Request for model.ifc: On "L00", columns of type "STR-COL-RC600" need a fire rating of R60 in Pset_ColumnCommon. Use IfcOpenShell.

First a look at what the model holds.

```python
import ifcopenshell
import ifcopenshell.util.element

model = ifcopenshell.open("model.ifc")
print(model.schema)
storey = next(s for s in model.by_type("IfcBuildingStorey") if s.Name == "L00")
columns = [e for e in ifcopenshell.util.element.get_decomposition(storey) if e.is_a("IfcColumn")]
seen = {}
for e in columns:
    element_type = ifcopenshell.util.element.get_type(e)
    key = (element_type.Name if element_type != e and element_type else None, ifcopenshell.util.element.get_pset(e, "Pset_ColumnCommon", "FireRating"))
    seen[key] = seen.get(key, 0) + 1
for (name, value), count in sorted(seen.items(), key=str):
    print(count, "x", name, "|", value)
```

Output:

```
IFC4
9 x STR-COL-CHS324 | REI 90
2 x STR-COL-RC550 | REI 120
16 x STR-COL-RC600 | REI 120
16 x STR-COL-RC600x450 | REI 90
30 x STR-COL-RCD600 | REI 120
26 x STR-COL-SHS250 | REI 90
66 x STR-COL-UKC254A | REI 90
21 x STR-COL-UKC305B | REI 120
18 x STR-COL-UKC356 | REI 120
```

```python
import ifcopenshell
import ifcopenshell.api.pset
import ifcopenshell.util.element

model = ifcopenshell.open("model.ifc")

storey = next(s for s in model.by_type("IfcBuildingStorey") if s.Name == "L00")
columns = [e for e in ifcopenshell.util.element.get_decomposition(storey) if e.is_a("IfcColumn")]

count = 0
for e in columns:
    element_type = ifcopenshell.util.element.get_type(e)
    if element_type in (None, e) or element_type.Name != "STR-COL-RC600":
        continue
    # add_pset returns the element's existing set when there is one.
    pset = ifcopenshell.api.pset.add_pset(model, product=e, name="Pset_ColumnCommon")
    ifcopenshell.api.pset.edit_pset(model, pset=pset, properties={"FireRating": "R60"})
    count += 1

print(count, "columns updated")

model.write("model_edited.ifc")
```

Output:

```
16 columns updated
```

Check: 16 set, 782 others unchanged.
